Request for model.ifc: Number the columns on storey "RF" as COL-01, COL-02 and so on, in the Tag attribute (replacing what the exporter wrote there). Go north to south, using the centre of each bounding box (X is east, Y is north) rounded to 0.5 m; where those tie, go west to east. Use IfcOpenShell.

First a look at what the model holds.

```python
import ifcopenshell
import ifcopenshell.util.element
import ifcopenshell.util.placement

model = ifcopenshell.open("model.ifc")
print(model.schema)
storey = next(s for s in model.by_type("IfcBuildingStorey") if s.Name == "RF")
columns = [e for e in ifcopenshell.util.element.get_decomposition(storey) if e.is_a("IfcColumn")]
for e in sorted(columns, key=lambda e: e.id()):
    origin = ifcopenshell.util.placement.get_local_placement(e.ObjectPlacement)[:3, 3]
    print(e.id(), e.Tag, e.Name, origin.round(2) + 0.0, sep=" | ")
```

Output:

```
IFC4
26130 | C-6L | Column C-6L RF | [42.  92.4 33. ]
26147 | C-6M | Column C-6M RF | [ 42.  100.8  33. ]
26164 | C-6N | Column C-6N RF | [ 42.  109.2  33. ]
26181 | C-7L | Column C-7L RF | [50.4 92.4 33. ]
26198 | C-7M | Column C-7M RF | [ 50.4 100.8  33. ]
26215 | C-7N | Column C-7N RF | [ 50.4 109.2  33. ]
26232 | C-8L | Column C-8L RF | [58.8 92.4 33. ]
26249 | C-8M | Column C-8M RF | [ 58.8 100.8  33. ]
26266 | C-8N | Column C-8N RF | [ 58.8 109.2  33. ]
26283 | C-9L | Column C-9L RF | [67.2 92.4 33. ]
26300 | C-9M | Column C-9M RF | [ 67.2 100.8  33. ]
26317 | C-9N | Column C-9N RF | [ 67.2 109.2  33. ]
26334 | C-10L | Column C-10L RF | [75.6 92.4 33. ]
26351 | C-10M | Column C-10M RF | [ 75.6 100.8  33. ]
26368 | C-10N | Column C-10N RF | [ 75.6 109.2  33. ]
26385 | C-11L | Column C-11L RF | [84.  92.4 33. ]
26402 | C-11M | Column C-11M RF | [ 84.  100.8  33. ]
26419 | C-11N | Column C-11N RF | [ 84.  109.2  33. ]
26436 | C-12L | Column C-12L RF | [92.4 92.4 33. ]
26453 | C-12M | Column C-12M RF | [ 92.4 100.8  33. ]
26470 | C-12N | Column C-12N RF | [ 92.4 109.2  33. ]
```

```python
import ifcopenshell
import ifcopenshell.geom
import ifcopenshell.util.element
import ifcopenshell.util.shape

model = ifcopenshell.open("model.ifc")
settings = ifcopenshell.geom.settings()
settings.set("use-world-coords", True)


def centre(element):
    shape = ifcopenshell.geom.create_shape(settings, element)
    return ifcopenshell.util.shape.get_bbox_centroid(shape.geometry)


storey = next(s for s in model.by_type("IfcBuildingStorey") if s.Name == "RF")
columns = [e for e in ifcopenshell.util.element.get_decomposition(storey) if e.is_a("IfcColumn")]

# Insertion points can sit at a corner or the storey origin, so sort by the geometry (in metres).
centres = {e: centre(e) for e in columns}
columns.sort(key=lambda e: (-round(centres[e][1] / 0.5), centres[e][0]))

for i, e in enumerate(columns, start=1):
    number = f"COL-{i:02d}"
    e.Tag = number
    print(e.id(), number)

model.write("model_edited.ifc")
```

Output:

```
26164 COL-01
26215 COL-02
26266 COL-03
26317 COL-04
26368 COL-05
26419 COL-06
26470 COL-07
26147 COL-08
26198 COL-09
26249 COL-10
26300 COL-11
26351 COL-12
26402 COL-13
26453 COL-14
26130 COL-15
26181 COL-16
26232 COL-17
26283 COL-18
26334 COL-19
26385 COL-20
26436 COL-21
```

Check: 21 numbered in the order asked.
